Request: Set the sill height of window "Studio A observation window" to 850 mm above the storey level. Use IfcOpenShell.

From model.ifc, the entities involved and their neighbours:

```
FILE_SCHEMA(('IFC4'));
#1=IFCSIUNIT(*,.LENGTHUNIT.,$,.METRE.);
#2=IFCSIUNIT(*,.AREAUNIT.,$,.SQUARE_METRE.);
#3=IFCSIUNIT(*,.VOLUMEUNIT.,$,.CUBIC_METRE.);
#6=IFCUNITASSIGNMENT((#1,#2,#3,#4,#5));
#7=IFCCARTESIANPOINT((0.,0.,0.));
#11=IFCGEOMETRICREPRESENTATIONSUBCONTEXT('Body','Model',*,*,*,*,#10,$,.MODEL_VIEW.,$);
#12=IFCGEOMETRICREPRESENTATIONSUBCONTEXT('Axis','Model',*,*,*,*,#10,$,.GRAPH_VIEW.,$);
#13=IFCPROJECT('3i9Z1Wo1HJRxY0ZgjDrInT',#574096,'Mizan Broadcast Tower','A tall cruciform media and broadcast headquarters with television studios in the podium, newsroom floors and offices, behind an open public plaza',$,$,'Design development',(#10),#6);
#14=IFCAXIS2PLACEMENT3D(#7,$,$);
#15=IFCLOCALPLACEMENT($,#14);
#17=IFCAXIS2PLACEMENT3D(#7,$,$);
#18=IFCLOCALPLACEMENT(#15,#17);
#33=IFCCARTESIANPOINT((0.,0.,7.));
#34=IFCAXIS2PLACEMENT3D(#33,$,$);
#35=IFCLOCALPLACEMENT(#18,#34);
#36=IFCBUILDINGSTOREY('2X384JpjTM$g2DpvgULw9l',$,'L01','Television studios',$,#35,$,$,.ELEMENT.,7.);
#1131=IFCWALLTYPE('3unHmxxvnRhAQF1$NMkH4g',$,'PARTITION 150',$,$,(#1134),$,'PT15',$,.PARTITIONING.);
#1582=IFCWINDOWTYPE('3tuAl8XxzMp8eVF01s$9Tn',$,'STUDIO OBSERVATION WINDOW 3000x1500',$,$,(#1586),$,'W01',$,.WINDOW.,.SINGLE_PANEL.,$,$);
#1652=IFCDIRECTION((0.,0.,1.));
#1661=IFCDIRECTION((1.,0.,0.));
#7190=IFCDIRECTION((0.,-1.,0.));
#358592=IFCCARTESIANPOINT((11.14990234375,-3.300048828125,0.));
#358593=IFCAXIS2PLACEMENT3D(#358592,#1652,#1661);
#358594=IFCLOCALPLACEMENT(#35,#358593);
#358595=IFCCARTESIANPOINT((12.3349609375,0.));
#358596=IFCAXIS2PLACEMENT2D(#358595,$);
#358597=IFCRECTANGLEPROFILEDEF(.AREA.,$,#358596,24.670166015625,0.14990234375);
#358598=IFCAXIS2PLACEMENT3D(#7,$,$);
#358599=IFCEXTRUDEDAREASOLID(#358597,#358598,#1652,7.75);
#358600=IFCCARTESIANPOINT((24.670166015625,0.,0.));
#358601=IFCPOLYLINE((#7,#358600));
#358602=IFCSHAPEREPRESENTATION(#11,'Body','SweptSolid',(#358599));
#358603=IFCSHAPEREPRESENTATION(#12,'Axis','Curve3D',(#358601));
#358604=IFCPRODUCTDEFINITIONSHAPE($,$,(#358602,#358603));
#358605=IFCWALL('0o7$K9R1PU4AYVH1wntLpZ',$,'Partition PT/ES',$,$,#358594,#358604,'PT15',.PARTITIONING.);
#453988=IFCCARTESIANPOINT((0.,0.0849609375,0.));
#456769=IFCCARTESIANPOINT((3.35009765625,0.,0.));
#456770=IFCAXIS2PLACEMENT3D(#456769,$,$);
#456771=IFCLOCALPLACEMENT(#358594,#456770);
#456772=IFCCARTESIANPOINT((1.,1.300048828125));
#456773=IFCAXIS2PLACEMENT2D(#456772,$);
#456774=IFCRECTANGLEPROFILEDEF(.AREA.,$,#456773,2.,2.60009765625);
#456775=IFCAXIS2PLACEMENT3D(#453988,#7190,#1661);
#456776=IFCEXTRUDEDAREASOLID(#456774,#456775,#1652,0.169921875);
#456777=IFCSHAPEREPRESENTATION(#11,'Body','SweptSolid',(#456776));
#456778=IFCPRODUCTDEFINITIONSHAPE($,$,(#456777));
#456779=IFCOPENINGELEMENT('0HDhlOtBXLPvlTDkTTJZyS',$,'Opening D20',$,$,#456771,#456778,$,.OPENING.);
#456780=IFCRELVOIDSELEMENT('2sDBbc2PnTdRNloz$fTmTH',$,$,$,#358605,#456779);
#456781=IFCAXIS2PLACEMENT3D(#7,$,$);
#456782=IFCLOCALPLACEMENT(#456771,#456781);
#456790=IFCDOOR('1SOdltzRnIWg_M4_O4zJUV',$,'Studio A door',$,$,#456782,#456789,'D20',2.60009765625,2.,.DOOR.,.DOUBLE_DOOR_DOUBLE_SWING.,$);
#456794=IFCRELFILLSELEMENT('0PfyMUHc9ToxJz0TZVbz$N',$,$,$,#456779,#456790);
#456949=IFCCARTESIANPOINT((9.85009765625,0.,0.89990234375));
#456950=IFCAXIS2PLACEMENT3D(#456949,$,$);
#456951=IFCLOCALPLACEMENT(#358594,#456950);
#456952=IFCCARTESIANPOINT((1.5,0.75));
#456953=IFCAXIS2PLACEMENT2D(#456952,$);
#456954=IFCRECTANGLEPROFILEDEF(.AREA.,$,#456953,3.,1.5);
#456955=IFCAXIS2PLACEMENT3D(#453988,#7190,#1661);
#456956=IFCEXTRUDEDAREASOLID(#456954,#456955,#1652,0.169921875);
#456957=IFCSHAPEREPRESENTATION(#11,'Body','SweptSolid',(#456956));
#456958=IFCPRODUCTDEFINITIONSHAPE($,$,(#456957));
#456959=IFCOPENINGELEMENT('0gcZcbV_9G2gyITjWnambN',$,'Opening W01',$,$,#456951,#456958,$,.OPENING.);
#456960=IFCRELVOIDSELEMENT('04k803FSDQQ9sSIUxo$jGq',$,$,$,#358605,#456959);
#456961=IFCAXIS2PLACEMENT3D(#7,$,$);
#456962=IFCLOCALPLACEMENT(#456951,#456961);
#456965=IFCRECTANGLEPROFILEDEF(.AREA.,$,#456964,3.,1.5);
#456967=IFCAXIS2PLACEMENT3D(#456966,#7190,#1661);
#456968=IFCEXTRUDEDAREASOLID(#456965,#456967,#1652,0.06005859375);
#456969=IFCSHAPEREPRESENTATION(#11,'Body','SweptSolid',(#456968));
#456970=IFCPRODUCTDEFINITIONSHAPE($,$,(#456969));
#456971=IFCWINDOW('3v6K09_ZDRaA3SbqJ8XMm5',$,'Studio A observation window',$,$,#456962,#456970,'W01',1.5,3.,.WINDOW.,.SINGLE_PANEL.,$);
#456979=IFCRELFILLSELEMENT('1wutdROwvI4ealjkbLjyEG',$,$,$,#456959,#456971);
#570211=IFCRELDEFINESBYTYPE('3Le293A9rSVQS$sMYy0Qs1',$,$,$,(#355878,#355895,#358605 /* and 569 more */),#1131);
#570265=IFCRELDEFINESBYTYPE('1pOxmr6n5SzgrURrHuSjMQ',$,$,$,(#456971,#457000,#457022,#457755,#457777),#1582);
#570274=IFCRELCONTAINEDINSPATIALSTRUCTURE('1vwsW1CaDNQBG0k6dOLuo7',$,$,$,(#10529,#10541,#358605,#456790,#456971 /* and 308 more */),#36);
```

```python
import numpy as np
import ifcopenshell
import ifcopenshell.api.geometry
import ifcopenshell.geom
import ifcopenshell.util.element
import ifcopenshell.util.placement
import ifcopenshell.util.shape
import ifcopenshell.util.unit

model = ifcopenshell.open("model.ifc")
unit_scale = ifcopenshell.util.unit.calculate_unit_scale(model)

window = model.by_id(456971)
opening = window.FillsVoids[0].RelatingOpeningElement
storey = ifcopenshell.util.element.get_container(window, ifc_class="IfcBuildingStorey")
level = ifcopenshell.util.placement.get_local_placement(storey.ObjectPlacement)[2, 3]

# The opening's origin need not be at the sill, so measure its lowest point.
shape = ifcopenshell.geom.create_shape(ifcopenshell.geom.settings(), opening)
bottom = ifcopenshell.util.shape.get_shape_bottom_elevation(shape, shape.geometry) / unit_scale
dz = level + 0.85 / unit_scale - bottom

shift = np.array([0.0, 0.0, dz])
# The window is placed relative to its opening, so it follows when the opening moves.
matrix = ifcopenshell.util.placement.get_local_placement(opening.ObjectPlacement)
matrix[:3, 3] += shift
ifcopenshell.api.geometry.edit_object_placement(
    model, product=opening, matrix=matrix, is_si=False, should_transform_children=True
)

print(f"moved by {dz * unit_scale:+.3f} m")

model.write("model_edited.ifc")
```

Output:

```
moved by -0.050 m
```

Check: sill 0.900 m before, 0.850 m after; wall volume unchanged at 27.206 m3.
